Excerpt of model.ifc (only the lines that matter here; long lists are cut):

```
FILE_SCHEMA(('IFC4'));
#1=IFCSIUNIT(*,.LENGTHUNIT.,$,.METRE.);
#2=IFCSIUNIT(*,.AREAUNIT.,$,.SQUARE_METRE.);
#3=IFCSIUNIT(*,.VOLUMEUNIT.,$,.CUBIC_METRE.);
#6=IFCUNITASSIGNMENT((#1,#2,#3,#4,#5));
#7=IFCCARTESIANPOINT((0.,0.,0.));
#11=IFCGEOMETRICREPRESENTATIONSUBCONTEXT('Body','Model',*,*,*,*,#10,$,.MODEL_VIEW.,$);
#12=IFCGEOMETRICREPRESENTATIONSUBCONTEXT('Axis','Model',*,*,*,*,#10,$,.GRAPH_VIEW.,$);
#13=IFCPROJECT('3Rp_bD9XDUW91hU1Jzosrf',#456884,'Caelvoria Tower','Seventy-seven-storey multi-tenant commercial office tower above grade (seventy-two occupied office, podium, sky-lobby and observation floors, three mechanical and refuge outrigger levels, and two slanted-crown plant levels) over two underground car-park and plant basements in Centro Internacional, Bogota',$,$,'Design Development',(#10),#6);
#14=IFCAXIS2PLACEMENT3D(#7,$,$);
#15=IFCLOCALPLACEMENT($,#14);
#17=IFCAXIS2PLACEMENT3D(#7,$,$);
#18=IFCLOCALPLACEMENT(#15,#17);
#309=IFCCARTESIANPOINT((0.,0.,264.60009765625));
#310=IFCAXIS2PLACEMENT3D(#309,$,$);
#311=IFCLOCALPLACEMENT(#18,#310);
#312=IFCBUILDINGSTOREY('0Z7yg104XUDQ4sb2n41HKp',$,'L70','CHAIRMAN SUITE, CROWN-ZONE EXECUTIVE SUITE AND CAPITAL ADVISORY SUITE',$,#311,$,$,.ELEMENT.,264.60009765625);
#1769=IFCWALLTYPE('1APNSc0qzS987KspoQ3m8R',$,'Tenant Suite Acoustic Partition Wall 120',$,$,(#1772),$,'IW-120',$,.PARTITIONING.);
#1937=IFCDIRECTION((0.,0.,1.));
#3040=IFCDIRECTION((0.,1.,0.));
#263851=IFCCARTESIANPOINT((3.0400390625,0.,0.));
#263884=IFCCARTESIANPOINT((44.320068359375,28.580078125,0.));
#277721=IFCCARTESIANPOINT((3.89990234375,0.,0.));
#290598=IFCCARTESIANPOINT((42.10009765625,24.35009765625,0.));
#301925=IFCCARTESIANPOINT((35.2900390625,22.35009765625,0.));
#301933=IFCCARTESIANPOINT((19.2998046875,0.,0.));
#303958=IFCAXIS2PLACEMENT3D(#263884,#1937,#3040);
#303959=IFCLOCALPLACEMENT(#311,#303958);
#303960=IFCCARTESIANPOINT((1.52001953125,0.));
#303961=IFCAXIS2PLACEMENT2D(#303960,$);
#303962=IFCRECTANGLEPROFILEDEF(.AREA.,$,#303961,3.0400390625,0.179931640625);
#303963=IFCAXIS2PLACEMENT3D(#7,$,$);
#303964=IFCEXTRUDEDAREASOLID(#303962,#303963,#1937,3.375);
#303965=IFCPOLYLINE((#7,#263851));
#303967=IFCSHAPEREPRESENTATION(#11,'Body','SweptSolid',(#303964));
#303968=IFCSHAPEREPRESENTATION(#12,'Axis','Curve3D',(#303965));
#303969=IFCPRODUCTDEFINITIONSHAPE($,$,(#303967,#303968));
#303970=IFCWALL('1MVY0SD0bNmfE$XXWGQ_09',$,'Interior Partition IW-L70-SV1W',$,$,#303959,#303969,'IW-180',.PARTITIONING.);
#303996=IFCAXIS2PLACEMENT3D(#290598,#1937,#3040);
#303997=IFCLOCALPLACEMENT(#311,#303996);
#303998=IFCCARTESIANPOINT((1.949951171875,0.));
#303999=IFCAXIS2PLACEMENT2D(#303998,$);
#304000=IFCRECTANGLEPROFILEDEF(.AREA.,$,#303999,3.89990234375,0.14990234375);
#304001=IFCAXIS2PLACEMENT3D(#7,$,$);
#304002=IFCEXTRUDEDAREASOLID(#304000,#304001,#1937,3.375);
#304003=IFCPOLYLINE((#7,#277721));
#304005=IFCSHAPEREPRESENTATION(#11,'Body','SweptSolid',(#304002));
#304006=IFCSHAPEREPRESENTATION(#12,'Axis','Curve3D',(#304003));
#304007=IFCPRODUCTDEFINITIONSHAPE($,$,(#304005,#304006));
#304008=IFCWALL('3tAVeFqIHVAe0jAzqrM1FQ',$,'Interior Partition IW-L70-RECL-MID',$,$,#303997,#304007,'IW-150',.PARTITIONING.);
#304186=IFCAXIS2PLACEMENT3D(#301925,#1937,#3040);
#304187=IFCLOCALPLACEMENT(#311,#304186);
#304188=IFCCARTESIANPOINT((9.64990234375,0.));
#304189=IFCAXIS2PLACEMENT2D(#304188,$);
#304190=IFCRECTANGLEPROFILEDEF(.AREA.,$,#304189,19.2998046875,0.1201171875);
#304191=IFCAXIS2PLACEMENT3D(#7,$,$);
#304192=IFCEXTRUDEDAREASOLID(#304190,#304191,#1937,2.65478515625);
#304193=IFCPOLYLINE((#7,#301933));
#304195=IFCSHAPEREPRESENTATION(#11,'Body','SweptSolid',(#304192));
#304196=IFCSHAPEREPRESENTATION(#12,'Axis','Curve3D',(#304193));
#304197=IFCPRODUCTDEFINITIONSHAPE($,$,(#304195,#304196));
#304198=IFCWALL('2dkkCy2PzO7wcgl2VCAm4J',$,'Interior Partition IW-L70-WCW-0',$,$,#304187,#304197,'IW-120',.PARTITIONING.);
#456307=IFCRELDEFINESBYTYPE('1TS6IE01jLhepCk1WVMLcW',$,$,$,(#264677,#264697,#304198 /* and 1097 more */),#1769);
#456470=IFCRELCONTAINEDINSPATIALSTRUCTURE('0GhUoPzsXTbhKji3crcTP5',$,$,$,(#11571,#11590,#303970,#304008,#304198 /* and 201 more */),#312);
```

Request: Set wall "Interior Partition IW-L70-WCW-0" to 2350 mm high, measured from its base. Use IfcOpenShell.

```python
import ifcopenshell
import ifcopenshell.geom
import ifcopenshell.util.representation
import ifcopenshell.util.shape
import ifcopenshell.util.unit

model = ifcopenshell.open("model.ifc")
unit_scale = ifcopenshell.util.unit.calculate_unit_scale(model)
settings = ifcopenshell.geom.settings()


def volume(element):
    """Net volume in cubic metres, openings subtracted."""
    shape = ifcopenshell.geom.create_shape(settings, element)
    return ifcopenshell.util.shape.get_volume(shape.geometry)


wall = model.by_id(304198)
before = volume(wall)

body = ifcopenshell.util.representation.get_representation(wall, "Model", "Body")
solid = body.Items[0]
old_height = solid.Depth
solid.Depth = 2.35 / unit_scale
after = volume(wall)

print(f"height {old_height:g} -> {solid.Depth:g}, volume {before:.3f} -> {after:.3f} m3")

model.write("model_v2.ifc")
```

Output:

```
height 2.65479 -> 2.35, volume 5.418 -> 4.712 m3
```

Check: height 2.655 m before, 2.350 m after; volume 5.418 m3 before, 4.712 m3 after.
